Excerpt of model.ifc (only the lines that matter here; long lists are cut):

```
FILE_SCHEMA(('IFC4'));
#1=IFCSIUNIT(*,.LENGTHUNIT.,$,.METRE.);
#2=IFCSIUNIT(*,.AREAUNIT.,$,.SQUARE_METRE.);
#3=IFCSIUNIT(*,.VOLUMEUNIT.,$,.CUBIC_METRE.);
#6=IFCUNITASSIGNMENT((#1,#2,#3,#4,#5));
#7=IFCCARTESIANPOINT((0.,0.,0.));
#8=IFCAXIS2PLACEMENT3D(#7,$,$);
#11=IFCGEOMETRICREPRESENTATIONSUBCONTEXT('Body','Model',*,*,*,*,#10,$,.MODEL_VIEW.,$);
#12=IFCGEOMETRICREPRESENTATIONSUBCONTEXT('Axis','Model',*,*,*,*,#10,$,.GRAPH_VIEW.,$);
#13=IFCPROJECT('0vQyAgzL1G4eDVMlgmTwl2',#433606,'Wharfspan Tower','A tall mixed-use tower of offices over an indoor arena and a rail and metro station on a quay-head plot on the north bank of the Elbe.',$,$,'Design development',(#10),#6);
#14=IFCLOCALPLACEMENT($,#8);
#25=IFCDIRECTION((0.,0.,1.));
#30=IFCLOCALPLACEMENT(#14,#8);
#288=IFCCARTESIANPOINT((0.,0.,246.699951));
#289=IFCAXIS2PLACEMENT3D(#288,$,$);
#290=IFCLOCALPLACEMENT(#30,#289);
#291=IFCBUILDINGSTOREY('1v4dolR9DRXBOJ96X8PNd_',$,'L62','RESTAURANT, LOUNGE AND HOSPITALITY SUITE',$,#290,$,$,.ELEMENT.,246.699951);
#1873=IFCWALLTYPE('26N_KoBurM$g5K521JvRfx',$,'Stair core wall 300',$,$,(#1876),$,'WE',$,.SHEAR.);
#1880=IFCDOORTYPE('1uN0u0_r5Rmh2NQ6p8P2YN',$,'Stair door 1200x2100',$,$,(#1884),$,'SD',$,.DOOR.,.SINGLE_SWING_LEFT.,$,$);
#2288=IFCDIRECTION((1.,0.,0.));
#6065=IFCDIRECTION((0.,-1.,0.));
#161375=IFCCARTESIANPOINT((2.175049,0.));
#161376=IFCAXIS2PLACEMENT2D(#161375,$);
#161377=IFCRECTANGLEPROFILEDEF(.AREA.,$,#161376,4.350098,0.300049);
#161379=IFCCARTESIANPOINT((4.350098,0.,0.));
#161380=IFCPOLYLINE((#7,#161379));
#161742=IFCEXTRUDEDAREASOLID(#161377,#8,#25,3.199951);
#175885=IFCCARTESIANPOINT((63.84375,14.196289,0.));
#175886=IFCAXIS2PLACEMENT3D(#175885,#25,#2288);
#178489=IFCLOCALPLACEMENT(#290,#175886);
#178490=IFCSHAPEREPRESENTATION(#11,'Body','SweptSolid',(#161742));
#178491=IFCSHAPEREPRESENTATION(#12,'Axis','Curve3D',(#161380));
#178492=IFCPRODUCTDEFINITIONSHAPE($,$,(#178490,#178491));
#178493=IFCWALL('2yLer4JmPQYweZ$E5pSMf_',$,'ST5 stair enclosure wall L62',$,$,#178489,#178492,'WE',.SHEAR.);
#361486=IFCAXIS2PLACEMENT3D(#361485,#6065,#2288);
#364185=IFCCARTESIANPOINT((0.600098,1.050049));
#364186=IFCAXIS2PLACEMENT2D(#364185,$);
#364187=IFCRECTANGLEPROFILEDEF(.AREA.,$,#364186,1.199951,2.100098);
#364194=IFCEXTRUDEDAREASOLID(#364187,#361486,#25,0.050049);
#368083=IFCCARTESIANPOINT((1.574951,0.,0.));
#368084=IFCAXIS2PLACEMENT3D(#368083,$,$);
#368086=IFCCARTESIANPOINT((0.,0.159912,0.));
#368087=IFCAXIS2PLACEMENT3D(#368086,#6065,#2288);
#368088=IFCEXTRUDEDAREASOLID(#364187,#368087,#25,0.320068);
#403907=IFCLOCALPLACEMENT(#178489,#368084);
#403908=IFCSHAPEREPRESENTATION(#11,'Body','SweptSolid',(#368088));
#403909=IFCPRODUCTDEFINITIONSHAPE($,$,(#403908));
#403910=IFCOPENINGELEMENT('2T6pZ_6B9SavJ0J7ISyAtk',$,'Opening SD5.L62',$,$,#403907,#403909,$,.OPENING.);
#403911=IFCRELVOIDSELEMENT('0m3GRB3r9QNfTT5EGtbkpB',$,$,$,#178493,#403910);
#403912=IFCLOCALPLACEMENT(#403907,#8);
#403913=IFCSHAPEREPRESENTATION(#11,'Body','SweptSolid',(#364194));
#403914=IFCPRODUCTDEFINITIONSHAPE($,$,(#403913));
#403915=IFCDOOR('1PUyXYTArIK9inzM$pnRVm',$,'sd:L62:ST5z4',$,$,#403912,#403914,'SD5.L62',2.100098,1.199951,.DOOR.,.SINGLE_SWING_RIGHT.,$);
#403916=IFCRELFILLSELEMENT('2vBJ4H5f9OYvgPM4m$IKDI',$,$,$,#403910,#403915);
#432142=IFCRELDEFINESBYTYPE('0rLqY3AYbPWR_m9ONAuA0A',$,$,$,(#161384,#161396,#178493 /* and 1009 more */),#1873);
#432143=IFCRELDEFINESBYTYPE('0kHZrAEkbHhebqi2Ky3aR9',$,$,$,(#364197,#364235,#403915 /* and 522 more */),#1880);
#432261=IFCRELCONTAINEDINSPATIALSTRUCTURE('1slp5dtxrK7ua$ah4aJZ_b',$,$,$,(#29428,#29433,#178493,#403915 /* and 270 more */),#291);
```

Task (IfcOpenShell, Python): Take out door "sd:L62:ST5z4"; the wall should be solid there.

```python
import ifcopenshell
import ifcopenshell.api.feature
import ifcopenshell.api.root
import ifcopenshell.geom
import ifcopenshell.util.shape

model = ifcopenshell.open("model.ifc")
settings = ifcopenshell.geom.settings()


def volume(element):
    """Net volume in cubic metres, openings subtracted."""
    shape = ifcopenshell.geom.create_shape(settings, element)
    return ifcopenshell.util.shape.get_volume(shape.geometry)


door = model.by_id(403915)
opening = door.FillsVoids[0].RelatingOpeningElement
wall = opening.VoidsElements[0].RelatingBuildingElement
before = volume(wall)

ifcopenshell.api.root.remove_product(model, product=door)
ifcopenshell.api.feature.remove_feature(model, feature=opening)

after = volume(wall)

print(f"wall volume {before:.3f} -> {after:.3f} m3")

model.write("model-out.ifc")
```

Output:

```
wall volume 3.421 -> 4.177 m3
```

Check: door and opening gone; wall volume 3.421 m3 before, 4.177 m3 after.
